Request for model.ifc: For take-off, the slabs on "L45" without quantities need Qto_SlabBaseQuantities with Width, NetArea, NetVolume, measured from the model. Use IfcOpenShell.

First a look at what the model holds.

```python
import ifcopenshell
import ifcopenshell.util.element
import ifcopenshell.util.unit

model = ifcopenshell.open("model.ifc")
print(model.schema)
for unit_type in ("LENGTHUNIT", "AREAUNIT", "VOLUMEUNIT"):
    print(unit_type, ifcopenshell.util.unit.calculate_unit_scale(model, unit_type))
storey = next(s for s in model.by_type("IfcBuildingStorey") if s.Name == "L45")
slabs = [e for e in ifcopenshell.util.element.get_decomposition(storey) if e.is_a("IfcSlab")]
for e in sorted(slabs, key=lambda e: e.id()):
    print(e.id(), e.is_a(), e.Name, list(ifcopenshell.util.element.get_psets(e, qtos_only=True)), sep=" | ")
```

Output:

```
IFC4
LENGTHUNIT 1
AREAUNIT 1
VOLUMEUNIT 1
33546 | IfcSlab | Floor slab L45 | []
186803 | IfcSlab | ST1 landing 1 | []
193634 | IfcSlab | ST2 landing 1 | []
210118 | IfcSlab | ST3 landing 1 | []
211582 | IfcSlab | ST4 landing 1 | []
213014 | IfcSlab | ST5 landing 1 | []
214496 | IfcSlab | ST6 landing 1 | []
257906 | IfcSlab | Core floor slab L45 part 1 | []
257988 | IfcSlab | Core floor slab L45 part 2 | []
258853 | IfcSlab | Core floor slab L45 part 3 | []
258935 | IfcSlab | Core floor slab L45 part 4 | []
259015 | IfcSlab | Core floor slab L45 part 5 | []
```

```python
import ifcopenshell
import ifcopenshell.api.pset
import ifcopenshell.geom
import ifcopenshell.util.element
import ifcopenshell.util.shape
import ifcopenshell.util.unit

model = ifcopenshell.open("model.ifc")
unit_scale = ifcopenshell.util.unit.calculate_unit_scale(model)
area_scale = ifcopenshell.util.unit.calculate_unit_scale(model, "AREAUNIT")
volume_scale = ifcopenshell.util.unit.calculate_unit_scale(model, "VOLUMEUNIT")
settings = ifcopenshell.geom.settings()

storey = next(s for s in model.by_type("IfcBuildingStorey") if s.Name == "L45")
slabs = [e for e in ifcopenshell.util.element.get_decomposition(storey) if e.is_a("IfcSlab")]

for e in sorted(slabs, key=lambda e: e.id()):
    if ifcopenshell.util.element.get_psets(e, qtos_only=True, should_inherit=False):
        continue
    # Geometry comes back in metres, in the element's own axes.
    shape = ifcopenshell.geom.create_shape(settings, e)
    values = {
        "Width": ifcopenshell.util.shape.get_z(shape.geometry) / unit_scale,
        "NetArea": ifcopenshell.util.shape.get_footprint_area(shape.geometry) / area_scale,
        "NetVolume": ifcopenshell.util.shape.get_volume(shape.geometry) / volume_scale,
    }
    qto = ifcopenshell.api.pset.add_qto(model, product=e, name="Qto_SlabBaseQuantities")
    ifcopenshell.api.pset.edit_qto(model, qto=qto, properties=values)
    print(e.id(), {k: round(v, 3) for k, v in values.items()})

model.write("model_rev.ifc")
```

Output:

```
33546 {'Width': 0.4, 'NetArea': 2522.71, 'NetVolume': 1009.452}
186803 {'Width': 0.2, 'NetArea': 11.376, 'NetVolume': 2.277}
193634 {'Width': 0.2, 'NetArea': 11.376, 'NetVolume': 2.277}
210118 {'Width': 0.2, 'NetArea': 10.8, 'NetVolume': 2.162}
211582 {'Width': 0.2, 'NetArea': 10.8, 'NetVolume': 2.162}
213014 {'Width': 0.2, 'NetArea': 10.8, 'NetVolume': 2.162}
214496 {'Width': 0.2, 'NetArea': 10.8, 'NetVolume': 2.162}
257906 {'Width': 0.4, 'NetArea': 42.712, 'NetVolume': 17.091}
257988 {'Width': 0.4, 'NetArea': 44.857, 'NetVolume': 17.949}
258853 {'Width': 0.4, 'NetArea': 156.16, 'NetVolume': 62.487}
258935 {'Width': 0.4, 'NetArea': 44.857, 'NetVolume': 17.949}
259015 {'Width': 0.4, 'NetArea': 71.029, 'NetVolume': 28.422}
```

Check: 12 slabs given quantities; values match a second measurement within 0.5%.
